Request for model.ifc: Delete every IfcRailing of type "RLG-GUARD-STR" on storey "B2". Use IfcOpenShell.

First a look at what the model holds.

```python
import ifcopenshell
import ifcopenshell.util.element

model = ifcopenshell.open("model.ifc")
print(model.schema)
storey = next(s for s in model.by_type("IfcBuildingStorey") if s.Name == "B2")
railings = [e for e in ifcopenshell.util.element.get_decomposition(storey) if e.is_a("IfcRailing")]
seen = {}
for e in railings:
    element_type = ifcopenshell.util.element.get_type(e)
    name = element_type.Name if element_type not in (None, e) else None
    seen[name] = seen.get(name, 0) + 1
for name, count in sorted(seen.items(), key=str):
    print(count, "x", name)
```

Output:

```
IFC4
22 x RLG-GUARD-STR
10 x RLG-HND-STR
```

```python
import ifcopenshell
import ifcopenshell.api.root
import ifcopenshell.util.element

model = ifcopenshell.open("model.ifc")

storey = next(s for s in model.by_type("IfcBuildingStorey") if s.Name == "B2")
railings = [e for e in ifcopenshell.util.element.get_decomposition(storey) if e.is_a("IfcRailing")]
targets = [e for e in railings if (t := ifcopenshell.util.element.get_type(e)) not in (None, e) and t.Name == "RLG-GUARD-STR"]

for e in targets:
    ifcopenshell.api.root.remove_product(model, product=e)
print(len(targets), "removed")

model.write("model_edited.ifc")
```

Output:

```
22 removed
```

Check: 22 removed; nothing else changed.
